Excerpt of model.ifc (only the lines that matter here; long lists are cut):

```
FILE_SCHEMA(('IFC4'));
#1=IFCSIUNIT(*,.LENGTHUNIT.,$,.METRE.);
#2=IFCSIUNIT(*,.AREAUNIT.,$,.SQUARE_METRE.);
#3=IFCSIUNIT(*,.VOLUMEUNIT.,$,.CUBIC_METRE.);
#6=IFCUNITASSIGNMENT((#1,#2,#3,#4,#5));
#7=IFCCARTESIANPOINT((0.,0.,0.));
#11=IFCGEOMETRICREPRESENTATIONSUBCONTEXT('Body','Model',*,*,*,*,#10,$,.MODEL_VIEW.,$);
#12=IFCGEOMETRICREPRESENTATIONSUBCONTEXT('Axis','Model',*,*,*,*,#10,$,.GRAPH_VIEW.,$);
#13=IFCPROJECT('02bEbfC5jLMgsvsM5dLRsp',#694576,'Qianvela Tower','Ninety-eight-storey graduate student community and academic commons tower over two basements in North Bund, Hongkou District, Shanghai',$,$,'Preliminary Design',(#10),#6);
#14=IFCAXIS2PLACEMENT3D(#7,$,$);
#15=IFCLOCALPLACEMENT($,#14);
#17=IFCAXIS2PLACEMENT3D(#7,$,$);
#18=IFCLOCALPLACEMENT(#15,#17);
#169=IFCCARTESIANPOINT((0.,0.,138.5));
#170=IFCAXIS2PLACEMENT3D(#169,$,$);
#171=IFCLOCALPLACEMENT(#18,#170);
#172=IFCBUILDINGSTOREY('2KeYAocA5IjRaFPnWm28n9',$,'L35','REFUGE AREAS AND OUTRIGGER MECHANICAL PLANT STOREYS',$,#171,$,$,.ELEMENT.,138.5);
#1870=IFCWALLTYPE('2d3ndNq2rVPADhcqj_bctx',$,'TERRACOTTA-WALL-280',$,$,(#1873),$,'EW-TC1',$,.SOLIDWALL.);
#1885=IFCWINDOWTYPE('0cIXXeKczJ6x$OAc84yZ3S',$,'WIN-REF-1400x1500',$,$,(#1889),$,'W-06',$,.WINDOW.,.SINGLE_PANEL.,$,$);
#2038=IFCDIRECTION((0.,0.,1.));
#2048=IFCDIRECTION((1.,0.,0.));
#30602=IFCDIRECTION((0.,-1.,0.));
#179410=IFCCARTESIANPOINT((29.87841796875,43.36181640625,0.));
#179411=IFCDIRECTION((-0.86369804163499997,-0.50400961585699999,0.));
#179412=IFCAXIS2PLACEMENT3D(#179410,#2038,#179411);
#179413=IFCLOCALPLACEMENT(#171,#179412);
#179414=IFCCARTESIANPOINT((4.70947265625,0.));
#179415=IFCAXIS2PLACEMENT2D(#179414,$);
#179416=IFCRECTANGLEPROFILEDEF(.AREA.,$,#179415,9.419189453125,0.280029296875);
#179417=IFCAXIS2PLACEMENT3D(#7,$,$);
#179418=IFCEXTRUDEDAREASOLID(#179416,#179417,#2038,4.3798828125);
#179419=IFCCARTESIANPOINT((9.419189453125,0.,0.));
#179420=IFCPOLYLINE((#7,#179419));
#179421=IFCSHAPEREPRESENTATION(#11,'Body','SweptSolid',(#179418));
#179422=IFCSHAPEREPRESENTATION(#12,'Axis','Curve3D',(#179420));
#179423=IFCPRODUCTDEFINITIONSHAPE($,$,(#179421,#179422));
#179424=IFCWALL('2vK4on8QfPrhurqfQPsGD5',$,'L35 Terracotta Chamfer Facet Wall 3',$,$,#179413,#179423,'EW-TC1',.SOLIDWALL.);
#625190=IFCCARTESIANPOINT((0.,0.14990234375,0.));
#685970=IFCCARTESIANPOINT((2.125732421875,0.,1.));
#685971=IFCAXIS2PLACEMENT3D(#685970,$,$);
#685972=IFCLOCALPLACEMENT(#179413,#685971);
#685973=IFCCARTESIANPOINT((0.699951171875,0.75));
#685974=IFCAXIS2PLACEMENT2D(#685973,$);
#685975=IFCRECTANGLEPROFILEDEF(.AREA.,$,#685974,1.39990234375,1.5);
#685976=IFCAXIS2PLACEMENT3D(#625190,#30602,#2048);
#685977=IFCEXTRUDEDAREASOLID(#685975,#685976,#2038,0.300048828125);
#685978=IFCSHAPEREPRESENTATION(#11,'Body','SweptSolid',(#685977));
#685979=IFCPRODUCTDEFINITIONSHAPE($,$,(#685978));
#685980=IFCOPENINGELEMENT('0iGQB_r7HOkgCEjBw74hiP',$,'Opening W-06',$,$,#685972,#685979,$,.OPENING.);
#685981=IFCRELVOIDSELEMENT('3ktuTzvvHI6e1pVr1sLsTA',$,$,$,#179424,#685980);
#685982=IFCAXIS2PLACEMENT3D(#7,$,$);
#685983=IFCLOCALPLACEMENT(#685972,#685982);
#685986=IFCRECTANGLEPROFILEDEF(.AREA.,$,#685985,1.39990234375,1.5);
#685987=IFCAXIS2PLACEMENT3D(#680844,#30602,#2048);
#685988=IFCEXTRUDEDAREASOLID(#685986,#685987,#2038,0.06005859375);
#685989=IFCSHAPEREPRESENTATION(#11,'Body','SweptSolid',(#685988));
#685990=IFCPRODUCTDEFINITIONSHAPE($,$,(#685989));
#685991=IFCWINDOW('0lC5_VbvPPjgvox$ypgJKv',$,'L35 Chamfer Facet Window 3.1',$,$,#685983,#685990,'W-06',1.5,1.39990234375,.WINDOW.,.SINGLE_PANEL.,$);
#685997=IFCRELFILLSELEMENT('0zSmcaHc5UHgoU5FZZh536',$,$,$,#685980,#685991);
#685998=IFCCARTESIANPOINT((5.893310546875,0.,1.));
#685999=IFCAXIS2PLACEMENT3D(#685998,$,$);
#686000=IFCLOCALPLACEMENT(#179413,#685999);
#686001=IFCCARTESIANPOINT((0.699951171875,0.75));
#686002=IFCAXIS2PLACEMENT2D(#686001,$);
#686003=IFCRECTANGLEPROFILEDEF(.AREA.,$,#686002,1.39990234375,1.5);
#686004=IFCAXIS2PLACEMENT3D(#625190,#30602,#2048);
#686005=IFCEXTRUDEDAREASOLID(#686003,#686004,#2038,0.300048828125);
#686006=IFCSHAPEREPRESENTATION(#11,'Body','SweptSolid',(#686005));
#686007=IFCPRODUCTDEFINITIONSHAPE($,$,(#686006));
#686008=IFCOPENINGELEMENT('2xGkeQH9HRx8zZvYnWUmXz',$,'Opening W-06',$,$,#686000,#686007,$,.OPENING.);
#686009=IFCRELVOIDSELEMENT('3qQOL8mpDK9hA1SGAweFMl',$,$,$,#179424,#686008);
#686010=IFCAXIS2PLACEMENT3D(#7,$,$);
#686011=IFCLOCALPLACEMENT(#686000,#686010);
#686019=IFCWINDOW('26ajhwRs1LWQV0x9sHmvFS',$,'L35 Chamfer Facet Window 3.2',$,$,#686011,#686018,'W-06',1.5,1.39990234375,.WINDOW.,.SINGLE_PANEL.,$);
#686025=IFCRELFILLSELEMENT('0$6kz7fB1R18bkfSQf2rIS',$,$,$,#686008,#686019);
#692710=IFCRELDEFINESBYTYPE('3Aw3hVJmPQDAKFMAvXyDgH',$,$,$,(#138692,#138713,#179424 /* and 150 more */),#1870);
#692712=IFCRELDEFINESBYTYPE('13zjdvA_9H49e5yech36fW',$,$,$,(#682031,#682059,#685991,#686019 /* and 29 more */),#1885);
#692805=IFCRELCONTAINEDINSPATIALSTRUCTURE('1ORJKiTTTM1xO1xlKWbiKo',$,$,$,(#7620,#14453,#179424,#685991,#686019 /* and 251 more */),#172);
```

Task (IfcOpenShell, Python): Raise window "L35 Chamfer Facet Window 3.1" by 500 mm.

```python
import numpy as np
import ifcopenshell
import ifcopenshell.api.geometry
import ifcopenshell.util.placement
import ifcopenshell.util.unit

model = ifcopenshell.open("model.ifc")
unit_scale = ifcopenshell.util.unit.calculate_unit_scale(model)

window = model.by_guid("0lC5_VbvPPjgvox$ypgJKv")
opening = window.FillsVoids[0].RelatingOpeningElement
dz = 0.5 / unit_scale

shift = np.array([0.0, 0.0, dz])
# The window is placed relative to its opening, so it follows when the opening moves.
matrix = ifcopenshell.util.placement.get_local_placement(opening.ObjectPlacement)
matrix[:3, 3] += shift
ifcopenshell.api.geometry.edit_object_placement(
    model, product=opening, matrix=matrix, is_si=False, should_transform_children=True
)

print(f"moved by {dz * unit_scale:+.3f} m")

model.write("model_rev.ifc")
```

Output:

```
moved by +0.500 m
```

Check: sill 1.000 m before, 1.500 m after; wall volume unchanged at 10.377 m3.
